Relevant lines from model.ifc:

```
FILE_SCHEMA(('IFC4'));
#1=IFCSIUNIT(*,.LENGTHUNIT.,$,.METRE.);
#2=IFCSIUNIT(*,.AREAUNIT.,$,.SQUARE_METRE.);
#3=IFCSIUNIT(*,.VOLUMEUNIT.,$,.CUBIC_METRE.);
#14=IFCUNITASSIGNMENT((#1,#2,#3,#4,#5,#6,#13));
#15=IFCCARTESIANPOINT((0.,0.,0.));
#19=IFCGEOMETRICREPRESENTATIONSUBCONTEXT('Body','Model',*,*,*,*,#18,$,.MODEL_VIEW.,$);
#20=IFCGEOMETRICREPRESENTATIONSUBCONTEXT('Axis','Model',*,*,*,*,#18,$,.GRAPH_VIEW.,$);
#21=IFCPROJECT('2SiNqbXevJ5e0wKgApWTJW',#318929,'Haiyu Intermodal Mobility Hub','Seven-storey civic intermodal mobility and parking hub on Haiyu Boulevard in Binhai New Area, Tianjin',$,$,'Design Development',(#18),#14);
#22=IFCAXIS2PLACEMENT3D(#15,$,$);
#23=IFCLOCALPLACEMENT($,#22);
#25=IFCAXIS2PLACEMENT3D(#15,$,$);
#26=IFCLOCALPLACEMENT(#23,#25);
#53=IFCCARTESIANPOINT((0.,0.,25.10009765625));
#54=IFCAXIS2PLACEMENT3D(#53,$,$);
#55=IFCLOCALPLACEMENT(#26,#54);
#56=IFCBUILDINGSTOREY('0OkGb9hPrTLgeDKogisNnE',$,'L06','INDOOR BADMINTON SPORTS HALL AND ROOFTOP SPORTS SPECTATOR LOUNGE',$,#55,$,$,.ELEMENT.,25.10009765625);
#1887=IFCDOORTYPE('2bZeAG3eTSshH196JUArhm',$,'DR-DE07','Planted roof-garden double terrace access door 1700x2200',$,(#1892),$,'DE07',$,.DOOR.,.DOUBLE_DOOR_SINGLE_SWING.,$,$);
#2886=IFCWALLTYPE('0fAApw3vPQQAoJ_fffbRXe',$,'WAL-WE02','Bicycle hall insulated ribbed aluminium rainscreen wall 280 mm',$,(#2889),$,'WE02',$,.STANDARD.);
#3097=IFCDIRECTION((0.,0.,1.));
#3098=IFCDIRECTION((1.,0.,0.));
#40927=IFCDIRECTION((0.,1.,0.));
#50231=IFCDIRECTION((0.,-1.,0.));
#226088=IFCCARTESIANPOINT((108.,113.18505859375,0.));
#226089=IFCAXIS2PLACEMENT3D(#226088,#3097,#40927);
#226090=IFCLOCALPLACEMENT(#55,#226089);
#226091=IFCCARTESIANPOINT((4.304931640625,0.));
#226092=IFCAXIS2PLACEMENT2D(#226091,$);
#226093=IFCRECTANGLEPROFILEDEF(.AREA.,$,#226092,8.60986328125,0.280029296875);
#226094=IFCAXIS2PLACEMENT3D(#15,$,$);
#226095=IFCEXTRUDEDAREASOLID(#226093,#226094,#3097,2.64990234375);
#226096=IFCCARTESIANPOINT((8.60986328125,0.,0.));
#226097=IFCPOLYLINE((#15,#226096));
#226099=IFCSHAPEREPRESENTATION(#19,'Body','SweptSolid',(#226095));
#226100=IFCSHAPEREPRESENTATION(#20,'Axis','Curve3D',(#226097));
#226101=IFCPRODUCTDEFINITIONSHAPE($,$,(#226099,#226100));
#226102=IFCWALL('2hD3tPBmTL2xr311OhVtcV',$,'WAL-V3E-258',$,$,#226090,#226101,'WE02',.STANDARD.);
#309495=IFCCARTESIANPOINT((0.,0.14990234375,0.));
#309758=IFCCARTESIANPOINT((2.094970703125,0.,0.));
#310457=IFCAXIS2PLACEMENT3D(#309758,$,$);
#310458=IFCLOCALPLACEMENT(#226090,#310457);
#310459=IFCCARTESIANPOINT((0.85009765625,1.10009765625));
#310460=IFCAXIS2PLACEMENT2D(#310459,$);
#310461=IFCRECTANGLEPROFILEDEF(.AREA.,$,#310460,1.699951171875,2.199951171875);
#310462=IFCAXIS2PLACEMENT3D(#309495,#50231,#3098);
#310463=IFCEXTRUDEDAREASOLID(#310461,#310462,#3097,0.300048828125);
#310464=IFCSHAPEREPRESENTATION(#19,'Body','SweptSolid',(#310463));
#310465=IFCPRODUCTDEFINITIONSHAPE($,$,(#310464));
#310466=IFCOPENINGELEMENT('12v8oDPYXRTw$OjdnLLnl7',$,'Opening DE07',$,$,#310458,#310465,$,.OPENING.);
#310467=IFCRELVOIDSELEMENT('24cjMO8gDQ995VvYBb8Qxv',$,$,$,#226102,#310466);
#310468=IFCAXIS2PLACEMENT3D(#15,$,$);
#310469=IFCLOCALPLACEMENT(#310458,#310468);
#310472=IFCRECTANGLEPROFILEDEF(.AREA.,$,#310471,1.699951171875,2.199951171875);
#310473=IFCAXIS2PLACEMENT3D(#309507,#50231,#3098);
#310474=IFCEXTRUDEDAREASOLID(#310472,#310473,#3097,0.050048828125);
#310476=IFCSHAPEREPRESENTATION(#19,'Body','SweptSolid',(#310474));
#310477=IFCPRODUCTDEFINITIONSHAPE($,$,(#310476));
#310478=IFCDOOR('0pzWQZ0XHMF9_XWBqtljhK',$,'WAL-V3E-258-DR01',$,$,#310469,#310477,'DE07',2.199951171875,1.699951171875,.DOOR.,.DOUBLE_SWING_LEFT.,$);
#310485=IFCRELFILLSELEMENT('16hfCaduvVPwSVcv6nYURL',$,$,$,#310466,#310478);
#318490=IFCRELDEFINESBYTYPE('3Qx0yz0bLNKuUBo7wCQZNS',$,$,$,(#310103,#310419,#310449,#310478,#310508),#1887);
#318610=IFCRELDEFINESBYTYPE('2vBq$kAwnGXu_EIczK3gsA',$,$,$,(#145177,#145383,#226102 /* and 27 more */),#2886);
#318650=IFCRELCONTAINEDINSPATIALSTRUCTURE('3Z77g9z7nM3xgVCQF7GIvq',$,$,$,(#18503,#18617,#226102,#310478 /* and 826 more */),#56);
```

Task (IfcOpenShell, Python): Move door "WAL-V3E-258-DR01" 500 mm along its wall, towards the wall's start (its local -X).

```python
import ifcopenshell
import ifcopenshell.api.geometry
import ifcopenshell.util.placement
import ifcopenshell.util.unit

model = ifcopenshell.open("model.ifc")
unit_scale = ifcopenshell.util.unit.calculate_unit_scale(model)

door = model.by_id(310478)
opening = door.FillsVoids[0].RelatingOpeningElement
wall = opening.VoidsElements[0].RelatingBuildingElement

wall_matrix = ifcopenshell.util.placement.get_local_placement(wall.ObjectPlacement)
shift = wall_matrix[:3, 0] * -0.5 / unit_scale
before = ifcopenshell.util.placement.get_local_placement(door.ObjectPlacement)[:3, 3].copy()

# The door is placed relative to its opening, so it follows when the opening moves.
matrix = ifcopenshell.util.placement.get_local_placement(opening.ObjectPlacement)
matrix[:3, 3] += shift
ifcopenshell.api.geometry.edit_object_placement(
    model, product=opening, matrix=matrix, is_si=False, should_transform_children=True
)

after = ifcopenshell.util.placement.get_local_placement(door.ObjectPlacement)[:3, 3]
print("door moved by", (after - before).round(3) + 0.0)

model.write("model-out.ifc")
```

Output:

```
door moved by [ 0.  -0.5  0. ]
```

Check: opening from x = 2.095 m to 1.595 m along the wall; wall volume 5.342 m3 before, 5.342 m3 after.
